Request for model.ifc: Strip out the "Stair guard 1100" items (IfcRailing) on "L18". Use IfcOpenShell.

First a look at what the model holds.

```python
import ifcopenshell
import ifcopenshell.util.element

model = ifcopenshell.open("model.ifc")
print(model.schema)
storey = next(s for s in model.by_type("IfcBuildingStorey") if s.Name == "L18")
railings = [e for e in ifcopenshell.util.element.get_decomposition(storey) if e.is_a("IfcRailing")]
seen = {}
for e in railings:
    element_type = ifcopenshell.util.element.get_type(e)
    name = element_type.Name if element_type not in (None, e) else None
    seen[name] = seen.get(name, 0) + 1
for name, count in sorted(seen.items(), key=str):
    print(count, "x", name)
```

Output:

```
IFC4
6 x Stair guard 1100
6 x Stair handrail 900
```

```python
import ifcopenshell
import ifcopenshell.api.root
import ifcopenshell.util.element

model = ifcopenshell.open("model.ifc")

storey = next(s for s in model.by_type("IfcBuildingStorey") if s.Name == "L18")
railings = [e for e in ifcopenshell.util.element.get_decomposition(storey) if e.is_a("IfcRailing")]
targets = [e for e in railings if (t := ifcopenshell.util.element.get_type(e)) not in (None, e) and t.Name == "Stair guard 1100"]

for e in targets:
    ifcopenshell.api.root.remove_product(model, product=e)
print(len(targets), "removed")

model.write("model_updated.ifc")
```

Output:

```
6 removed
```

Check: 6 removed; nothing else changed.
